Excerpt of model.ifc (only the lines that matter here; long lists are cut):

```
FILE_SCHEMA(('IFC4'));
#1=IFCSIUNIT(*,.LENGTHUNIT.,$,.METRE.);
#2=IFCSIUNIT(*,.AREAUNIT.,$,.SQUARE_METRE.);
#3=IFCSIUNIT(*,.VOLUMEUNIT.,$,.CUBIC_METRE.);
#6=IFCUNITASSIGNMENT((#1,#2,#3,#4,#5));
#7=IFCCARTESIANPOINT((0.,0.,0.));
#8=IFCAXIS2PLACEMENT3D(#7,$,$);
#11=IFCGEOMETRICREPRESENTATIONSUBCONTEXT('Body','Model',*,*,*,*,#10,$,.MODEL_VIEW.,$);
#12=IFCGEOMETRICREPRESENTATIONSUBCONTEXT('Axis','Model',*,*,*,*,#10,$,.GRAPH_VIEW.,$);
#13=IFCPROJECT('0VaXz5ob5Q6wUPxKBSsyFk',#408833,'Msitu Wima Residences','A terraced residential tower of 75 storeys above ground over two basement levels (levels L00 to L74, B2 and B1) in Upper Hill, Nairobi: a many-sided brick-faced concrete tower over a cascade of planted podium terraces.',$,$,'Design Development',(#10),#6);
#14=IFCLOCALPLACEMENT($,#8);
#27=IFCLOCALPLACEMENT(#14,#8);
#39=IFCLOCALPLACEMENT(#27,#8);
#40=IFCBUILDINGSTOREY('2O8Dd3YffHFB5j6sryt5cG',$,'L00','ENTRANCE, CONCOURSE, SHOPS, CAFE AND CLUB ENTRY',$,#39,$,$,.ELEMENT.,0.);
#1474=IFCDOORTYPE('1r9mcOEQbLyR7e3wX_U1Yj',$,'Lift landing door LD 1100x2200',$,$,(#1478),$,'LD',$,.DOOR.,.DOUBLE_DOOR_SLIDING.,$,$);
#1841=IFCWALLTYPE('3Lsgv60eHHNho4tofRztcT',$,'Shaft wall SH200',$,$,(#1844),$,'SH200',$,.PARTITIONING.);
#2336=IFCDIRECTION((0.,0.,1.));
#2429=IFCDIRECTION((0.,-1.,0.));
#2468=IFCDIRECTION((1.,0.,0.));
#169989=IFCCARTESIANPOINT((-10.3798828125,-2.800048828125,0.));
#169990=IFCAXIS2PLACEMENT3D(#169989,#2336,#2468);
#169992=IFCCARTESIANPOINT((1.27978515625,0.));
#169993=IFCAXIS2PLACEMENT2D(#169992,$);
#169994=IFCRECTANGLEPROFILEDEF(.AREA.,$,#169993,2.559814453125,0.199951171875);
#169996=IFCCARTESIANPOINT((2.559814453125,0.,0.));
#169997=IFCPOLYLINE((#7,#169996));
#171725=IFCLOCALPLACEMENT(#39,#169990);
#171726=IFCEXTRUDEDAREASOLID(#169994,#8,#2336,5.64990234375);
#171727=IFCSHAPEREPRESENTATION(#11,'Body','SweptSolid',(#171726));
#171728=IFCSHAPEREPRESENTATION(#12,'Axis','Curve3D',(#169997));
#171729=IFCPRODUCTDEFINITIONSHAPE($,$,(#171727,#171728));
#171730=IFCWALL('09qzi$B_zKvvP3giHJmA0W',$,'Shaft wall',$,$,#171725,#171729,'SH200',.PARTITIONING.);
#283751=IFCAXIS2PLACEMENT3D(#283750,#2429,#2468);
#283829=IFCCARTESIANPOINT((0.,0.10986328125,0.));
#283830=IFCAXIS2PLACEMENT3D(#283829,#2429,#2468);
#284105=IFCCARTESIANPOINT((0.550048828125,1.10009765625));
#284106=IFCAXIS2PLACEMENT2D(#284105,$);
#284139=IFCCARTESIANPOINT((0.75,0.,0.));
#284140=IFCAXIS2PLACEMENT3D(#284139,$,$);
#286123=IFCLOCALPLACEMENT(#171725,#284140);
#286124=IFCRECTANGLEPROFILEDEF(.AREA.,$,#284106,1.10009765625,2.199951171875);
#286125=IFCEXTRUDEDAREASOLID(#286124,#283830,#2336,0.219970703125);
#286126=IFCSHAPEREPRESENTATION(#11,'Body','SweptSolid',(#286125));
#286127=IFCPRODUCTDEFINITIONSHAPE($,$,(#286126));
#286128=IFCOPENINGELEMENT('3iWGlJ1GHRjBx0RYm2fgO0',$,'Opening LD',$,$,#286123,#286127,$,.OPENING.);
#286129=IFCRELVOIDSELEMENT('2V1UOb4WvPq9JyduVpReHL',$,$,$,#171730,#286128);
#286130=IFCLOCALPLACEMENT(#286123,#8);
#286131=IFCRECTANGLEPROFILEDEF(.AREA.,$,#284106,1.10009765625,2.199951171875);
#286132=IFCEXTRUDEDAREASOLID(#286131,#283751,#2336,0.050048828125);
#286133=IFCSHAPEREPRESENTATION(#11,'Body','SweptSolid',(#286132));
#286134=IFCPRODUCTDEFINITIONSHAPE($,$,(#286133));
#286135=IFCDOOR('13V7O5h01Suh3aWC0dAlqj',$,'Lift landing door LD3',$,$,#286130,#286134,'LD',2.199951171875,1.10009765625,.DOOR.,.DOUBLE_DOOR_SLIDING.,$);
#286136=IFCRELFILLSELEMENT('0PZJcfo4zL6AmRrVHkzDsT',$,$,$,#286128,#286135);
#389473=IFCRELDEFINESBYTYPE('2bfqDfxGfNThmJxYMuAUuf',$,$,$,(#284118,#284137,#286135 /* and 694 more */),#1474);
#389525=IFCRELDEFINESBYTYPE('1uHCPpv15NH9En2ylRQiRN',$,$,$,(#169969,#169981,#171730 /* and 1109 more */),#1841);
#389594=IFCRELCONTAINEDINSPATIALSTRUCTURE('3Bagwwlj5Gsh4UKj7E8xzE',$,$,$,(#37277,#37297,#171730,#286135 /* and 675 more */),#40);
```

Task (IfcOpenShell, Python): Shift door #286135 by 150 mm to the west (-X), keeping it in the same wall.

```python
import ifcopenshell
import ifcopenshell.api.geometry
import ifcopenshell.util.placement
import ifcopenshell.util.unit

model = ifcopenshell.open("model.ifc")
unit_scale = ifcopenshell.util.unit.calculate_unit_scale(model)

door = model.by_guid("13V7O5h01Suh3aWC0dAlqj")
opening = door.FillsVoids[0].RelatingOpeningElement
wall = opening.VoidsElements[0].RelatingBuildingElement

wall_matrix = ifcopenshell.util.placement.get_local_placement(wall.ObjectPlacement)
shift = wall_matrix[:3, 0] * -0.15 / unit_scale
before = ifcopenshell.util.placement.get_local_placement(door.ObjectPlacement)[:3, 3].copy()

# The door is placed relative to its opening, so it follows when the opening moves.
matrix = ifcopenshell.util.placement.get_local_placement(opening.ObjectPlacement)
matrix[:3, 3] += shift
ifcopenshell.api.geometry.edit_object_placement(
    model, product=opening, matrix=matrix, is_si=False, should_transform_children=True
)

after = ifcopenshell.util.placement.get_local_placement(door.ObjectPlacement)[:3, 3]
print("door moved by", (after - before).round(3) + 0.0)

model.write("model-out.ifc")
```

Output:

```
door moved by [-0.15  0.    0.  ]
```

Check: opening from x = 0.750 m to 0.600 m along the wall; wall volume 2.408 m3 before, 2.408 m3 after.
